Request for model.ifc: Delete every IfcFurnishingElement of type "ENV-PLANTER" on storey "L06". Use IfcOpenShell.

First a look at what the model holds.

```python
import ifcopenshell
import ifcopenshell.util.element

model = ifcopenshell.open("model.ifc")
print(model.schema)
storey = next(s for s in model.by_type("IfcBuildingStorey") if s.Name == "L06")
furniture = [e for e in ifcopenshell.util.element.get_decomposition(storey) if e.is_a("IfcFurnishingElement")]
seen = {}
for e in furniture:
    element_type = ifcopenshell.util.element.get_type(e)
    name = element_type.Name if element_type not in (None, e) else None
    seen[name] = seen.get(name, 0) + 1
for name, count in sorted(seen.items(), key=str):
    print(count, "x", name)
```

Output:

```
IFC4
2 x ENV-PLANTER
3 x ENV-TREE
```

```python
import ifcopenshell
import ifcopenshell.api.root
import ifcopenshell.util.element

model = ifcopenshell.open("model.ifc")

storey = next(s for s in model.by_type("IfcBuildingStorey") if s.Name == "L06")
furniture = [e for e in ifcopenshell.util.element.get_decomposition(storey) if e.is_a("IfcFurnishingElement")]
targets = [e for e in furniture if (t := ifcopenshell.util.element.get_type(e)) not in (None, e) and t.Name == "ENV-PLANTER"]

for e in targets:
    ifcopenshell.api.root.remove_product(model, product=e)
print(len(targets), "removed")

model.write("model_updated.ifc")
```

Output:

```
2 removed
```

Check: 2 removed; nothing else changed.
